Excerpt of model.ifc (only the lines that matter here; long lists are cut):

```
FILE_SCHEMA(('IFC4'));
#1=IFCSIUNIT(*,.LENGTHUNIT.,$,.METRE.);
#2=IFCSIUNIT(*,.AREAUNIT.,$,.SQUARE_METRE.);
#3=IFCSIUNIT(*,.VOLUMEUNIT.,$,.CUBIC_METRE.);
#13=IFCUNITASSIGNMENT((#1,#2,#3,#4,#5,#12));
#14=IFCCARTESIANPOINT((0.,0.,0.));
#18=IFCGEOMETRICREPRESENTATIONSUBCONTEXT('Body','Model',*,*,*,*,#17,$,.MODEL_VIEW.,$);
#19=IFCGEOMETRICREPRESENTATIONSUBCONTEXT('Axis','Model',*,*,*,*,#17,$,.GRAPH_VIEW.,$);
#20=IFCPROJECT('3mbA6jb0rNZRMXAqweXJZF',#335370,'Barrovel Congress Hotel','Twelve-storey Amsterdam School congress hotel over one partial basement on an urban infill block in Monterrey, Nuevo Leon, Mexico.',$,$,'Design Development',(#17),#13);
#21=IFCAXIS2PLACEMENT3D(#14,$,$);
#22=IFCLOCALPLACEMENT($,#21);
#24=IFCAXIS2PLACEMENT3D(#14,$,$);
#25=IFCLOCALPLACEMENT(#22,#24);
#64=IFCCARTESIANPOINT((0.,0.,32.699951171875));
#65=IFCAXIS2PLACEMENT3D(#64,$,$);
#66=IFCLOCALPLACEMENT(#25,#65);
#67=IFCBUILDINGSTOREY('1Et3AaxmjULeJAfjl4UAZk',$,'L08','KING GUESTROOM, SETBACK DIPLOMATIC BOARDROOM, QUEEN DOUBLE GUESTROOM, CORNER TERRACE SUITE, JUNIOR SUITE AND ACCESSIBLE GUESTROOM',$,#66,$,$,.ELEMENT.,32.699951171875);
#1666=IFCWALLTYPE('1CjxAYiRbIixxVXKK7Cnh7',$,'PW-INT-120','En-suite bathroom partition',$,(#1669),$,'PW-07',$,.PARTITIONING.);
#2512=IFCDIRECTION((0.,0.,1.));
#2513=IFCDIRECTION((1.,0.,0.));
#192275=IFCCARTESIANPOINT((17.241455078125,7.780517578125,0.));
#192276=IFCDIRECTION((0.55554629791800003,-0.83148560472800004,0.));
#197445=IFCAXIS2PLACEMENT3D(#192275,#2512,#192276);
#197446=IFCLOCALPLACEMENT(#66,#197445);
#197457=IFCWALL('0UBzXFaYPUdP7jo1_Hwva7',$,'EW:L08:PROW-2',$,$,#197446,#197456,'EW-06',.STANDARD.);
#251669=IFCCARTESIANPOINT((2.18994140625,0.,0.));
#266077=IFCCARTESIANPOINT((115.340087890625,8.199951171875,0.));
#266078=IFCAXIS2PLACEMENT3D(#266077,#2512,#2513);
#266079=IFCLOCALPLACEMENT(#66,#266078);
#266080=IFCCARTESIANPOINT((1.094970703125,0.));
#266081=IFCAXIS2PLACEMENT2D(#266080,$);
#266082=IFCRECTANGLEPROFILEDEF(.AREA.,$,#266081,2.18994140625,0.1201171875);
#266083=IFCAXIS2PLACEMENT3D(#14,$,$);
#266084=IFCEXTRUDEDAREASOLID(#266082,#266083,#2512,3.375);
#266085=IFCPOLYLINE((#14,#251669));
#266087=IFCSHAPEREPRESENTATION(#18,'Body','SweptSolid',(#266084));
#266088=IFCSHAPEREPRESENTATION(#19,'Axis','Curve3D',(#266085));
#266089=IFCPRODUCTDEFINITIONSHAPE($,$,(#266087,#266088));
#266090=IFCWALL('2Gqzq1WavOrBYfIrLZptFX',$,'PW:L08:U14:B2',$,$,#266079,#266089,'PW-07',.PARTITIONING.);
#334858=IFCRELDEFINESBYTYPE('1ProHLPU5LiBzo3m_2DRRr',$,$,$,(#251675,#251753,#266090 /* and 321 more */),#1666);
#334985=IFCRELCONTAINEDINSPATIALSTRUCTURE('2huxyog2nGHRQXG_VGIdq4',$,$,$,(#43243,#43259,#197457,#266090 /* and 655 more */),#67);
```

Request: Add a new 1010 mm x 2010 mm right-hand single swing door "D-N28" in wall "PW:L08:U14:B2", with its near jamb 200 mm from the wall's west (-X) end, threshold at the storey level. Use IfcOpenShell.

```python
import numpy as np
import ifcopenshell
import ifcopenshell.api.feature
import ifcopenshell.api.geometry
import ifcopenshell.api.root
import ifcopenshell.api.spatial
import ifcopenshell.geom
import ifcopenshell.util.element
import ifcopenshell.util.placement
import ifcopenshell.util.representation
import ifcopenshell.util.shape
import ifcopenshell.util.unit

model = ifcopenshell.open("model.ifc")
unit_scale = ifcopenshell.util.unit.calculate_unit_scale(model)
settings = ifcopenshell.geom.settings()


def volume(element):
    """Net volume in cubic metres, openings subtracted."""
    shape = ifcopenshell.geom.create_shape(settings, element)
    return ifcopenshell.util.shape.get_volume(shape.geometry)


wall = model.by_id(266090)
storey = ifcopenshell.util.element.get_container(wall, ifc_class="IfcBuildingStorey")
context = ifcopenshell.util.representation.get_context(model, "Model", "Body", "MODEL_VIEW")
before = volume(wall)

width, height, from_end, sill = 1.01, 2.01, 0.2, 0.0  # metres

# The wall runs along its own X axis, and the end named is its -X end.
wall_shape = ifcopenshell.geom.create_shape(settings, wall)
x, y, z = ifcopenshell.util.shape.get_vertices(wall_shape.geometry).T
start = x.min() + from_end
face, thickness = float(y.min()), float(y.max() - y.min())
wall_matrix = ifcopenshell.util.placement.get_local_placement(wall.ObjectPlacement)
level = ifcopenshell.util.placement.get_local_placement(storey.ObjectPlacement)[2, 3]


def in_wall(x, y):
    """Placement at x, y metres in the wall's axes, at sill height."""
    matrix = wall_matrix.copy()
    matrix[:, 3] = wall_matrix @ np.array([x / unit_scale, y / unit_scale, 0.0, 1.0])
    matrix[2, 3] = level + sill / unit_scale
    return matrix


# Opening: a box that overshoots both wall faces by 50 mm.
opening = ifcopenshell.api.root.create_entity(model, ifc_class="IfcOpeningElement", predefined_type="OPENING")
box = ifcopenshell.api.geometry.add_wall_representation(
    model, context=context, length=width, height=height, thickness=thickness + 0.1
)
ifcopenshell.api.geometry.assign_representation(model, product=opening, representation=box)
ifcopenshell.api.geometry.edit_object_placement(model, product=opening, matrix=in_wall(start, face - 0.05), is_si=False)
ifcopenshell.api.feature.add_feature(model, feature=opening, element=wall)

door = ifcopenshell.api.root.create_entity(model, ifc_class="IfcDoor", name="D-N28", predefined_type="DOOR")
door.OverallWidth, door.OverallHeight = width / unit_scale, height / unit_scale
door.OperationType = "SINGLE_SWING_RIGHT"
body = ifcopenshell.api.geometry.add_door_representation(
    model,
    context=context,
    overall_width=door.OverallWidth,
    overall_height=door.OverallHeight,
    operation_type="SINGLE_SWING_RIGHT",
    lining_properties={"LiningDepth": thickness / unit_scale, "ThresholdDepth": thickness / unit_scale},
)
ifcopenshell.api.geometry.assign_representation(model, product=door, representation=body)
ifcopenshell.api.spatial.assign_container(model, products=[door], relating_structure=storey)
ifcopenshell.api.feature.add_filling(model, opening=opening, element=door)

# The lining spans the wall, so the door starts at the wall face.
ifcopenshell.api.geometry.edit_object_placement(model, product=door, matrix=in_wall(start, face), is_si=False)

after = volume(wall)

print(f"wall volume {before:.3f} -> {after:.3f} m3")

model.write("model_rev.ifc")
```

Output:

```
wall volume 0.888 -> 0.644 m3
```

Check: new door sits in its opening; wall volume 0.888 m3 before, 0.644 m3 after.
